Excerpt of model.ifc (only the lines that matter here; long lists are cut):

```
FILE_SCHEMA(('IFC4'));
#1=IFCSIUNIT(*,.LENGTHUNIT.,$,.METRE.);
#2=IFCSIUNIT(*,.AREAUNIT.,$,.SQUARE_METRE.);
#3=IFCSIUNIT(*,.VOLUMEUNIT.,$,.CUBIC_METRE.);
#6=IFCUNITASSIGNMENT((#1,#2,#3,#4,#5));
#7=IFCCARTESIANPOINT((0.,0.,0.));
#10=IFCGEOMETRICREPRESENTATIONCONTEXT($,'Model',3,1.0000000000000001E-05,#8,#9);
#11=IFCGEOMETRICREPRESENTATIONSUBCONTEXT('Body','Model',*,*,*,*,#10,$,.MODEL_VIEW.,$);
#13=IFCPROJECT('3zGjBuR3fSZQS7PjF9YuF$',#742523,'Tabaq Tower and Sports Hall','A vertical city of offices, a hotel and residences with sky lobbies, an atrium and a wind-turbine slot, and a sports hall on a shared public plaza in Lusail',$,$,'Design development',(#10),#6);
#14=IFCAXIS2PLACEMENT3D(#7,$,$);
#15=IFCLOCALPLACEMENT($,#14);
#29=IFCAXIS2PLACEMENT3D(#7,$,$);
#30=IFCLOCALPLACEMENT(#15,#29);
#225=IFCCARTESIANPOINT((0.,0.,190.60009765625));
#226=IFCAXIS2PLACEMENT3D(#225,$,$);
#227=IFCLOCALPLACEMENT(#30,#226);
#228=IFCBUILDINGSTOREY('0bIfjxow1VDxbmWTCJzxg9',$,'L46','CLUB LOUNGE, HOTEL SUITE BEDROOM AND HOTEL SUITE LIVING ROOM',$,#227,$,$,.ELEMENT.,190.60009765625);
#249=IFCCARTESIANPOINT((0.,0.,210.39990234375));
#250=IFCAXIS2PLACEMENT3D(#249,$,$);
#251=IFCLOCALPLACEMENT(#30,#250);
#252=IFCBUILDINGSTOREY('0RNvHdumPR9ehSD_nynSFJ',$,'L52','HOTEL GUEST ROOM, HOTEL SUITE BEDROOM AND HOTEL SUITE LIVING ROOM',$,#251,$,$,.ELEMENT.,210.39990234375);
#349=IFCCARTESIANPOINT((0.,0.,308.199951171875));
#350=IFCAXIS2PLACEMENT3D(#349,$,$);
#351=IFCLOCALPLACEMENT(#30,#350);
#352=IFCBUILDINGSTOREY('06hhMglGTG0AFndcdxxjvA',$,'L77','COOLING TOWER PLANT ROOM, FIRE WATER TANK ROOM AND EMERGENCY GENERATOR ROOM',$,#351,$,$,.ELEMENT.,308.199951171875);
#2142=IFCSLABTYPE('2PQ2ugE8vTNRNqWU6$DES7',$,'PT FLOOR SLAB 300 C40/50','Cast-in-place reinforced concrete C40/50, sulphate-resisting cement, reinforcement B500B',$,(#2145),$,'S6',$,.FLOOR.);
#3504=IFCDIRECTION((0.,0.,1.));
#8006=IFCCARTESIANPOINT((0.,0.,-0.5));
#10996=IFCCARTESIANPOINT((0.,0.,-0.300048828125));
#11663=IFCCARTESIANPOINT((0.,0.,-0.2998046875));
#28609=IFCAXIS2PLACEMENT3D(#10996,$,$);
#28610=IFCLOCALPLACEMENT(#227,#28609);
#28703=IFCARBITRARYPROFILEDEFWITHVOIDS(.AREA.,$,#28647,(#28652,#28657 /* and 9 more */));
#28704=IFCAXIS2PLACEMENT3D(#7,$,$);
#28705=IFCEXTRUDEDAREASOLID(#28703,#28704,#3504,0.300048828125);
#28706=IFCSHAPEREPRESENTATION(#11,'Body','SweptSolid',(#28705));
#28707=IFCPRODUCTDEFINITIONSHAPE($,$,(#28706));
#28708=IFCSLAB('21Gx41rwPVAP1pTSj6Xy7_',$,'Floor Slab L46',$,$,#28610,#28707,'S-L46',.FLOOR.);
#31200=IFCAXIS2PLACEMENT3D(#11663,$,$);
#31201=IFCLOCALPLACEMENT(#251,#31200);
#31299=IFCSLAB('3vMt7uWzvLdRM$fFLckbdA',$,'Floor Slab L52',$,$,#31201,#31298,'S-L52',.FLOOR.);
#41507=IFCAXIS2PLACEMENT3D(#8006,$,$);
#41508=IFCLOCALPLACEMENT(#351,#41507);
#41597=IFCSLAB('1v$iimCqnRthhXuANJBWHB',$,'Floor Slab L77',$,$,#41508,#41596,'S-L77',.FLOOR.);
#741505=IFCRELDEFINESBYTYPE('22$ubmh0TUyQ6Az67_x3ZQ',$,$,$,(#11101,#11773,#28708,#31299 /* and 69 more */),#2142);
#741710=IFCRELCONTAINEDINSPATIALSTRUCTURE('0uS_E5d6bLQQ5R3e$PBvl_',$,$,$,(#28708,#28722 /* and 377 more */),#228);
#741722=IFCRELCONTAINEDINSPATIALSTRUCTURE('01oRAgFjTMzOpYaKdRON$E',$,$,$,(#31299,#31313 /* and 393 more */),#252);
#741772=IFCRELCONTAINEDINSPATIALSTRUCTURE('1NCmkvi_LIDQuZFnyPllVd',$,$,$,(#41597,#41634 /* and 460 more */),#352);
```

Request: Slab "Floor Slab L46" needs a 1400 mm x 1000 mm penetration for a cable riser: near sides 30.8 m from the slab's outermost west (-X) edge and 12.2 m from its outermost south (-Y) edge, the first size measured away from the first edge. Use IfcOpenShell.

```python
import numpy as np
import ifcopenshell
import ifcopenshell.api.feature
import ifcopenshell.api.geometry
import ifcopenshell.api.root
import ifcopenshell.geom
import ifcopenshell.util.placement
import ifcopenshell.util.representation
import ifcopenshell.util.shape
import ifcopenshell.util.unit

model = ifcopenshell.open("model.ifc")
unit_scale = ifcopenshell.util.unit.calculate_unit_scale(model)
settings = ifcopenshell.geom.settings()


def volume(element):
    """Net volume in cubic metres, openings subtracted."""
    shape = ifcopenshell.geom.create_shape(settings, element)
    return ifcopenshell.util.shape.get_volume(shape.geometry)


slab = model.by_guid("21Gx41rwPVAP1pTSj6Xy7_")
before = volume(slab)

# Extent in the slab's own axes, in metres. The edges named are its -X and -Y sides.
slab_shape = ifcopenshell.geom.create_shape(settings, slab)
vertices = ifcopenshell.util.shape.get_vertices(slab_shape.geometry)
x_min, y_min, bottom = vertices.min(axis=0)
top = vertices[:, 2].max()

opening = ifcopenshell.api.root.create_entity(model, ifc_class="IfcOpeningElement", name="Cable riser opening", predefined_type="OPENING")
context = ifcopenshell.util.representation.get_context(model, "Model", "Body", "MODEL_VIEW")
width, depth = 1.4, 1
outline = [(0.0, 0.0), (width, 0.0), (width, depth), (0.0, depth), (0.0, 0.0)]
# Overshoot both faces by 50 mm so the cut is clean.
shape = ifcopenshell.api.geometry.add_slab_representation(
    model, context=context, depth=top - bottom + 0.1, polyline=outline
)
ifcopenshell.api.geometry.assign_representation(model, product=opening, representation=shape)

matrix = ifcopenshell.util.placement.get_local_placement(slab.ObjectPlacement)
matrix[:, 3] = matrix @ np.append(np.array([x_min + 30.8, y_min + 12.2, bottom - 0.05]) / unit_scale, 1.0)
ifcopenshell.api.geometry.edit_object_placement(model, product=opening, matrix=matrix, is_si=False)
ifcopenshell.api.feature.add_feature(model, feature=opening, element=slab)

after = volume(slab)

print(f"slab volume {before:.3f} -> {after:.3f} m3")

model.write("model-out.ifc")
```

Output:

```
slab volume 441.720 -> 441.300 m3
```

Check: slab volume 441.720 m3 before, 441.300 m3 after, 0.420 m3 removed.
